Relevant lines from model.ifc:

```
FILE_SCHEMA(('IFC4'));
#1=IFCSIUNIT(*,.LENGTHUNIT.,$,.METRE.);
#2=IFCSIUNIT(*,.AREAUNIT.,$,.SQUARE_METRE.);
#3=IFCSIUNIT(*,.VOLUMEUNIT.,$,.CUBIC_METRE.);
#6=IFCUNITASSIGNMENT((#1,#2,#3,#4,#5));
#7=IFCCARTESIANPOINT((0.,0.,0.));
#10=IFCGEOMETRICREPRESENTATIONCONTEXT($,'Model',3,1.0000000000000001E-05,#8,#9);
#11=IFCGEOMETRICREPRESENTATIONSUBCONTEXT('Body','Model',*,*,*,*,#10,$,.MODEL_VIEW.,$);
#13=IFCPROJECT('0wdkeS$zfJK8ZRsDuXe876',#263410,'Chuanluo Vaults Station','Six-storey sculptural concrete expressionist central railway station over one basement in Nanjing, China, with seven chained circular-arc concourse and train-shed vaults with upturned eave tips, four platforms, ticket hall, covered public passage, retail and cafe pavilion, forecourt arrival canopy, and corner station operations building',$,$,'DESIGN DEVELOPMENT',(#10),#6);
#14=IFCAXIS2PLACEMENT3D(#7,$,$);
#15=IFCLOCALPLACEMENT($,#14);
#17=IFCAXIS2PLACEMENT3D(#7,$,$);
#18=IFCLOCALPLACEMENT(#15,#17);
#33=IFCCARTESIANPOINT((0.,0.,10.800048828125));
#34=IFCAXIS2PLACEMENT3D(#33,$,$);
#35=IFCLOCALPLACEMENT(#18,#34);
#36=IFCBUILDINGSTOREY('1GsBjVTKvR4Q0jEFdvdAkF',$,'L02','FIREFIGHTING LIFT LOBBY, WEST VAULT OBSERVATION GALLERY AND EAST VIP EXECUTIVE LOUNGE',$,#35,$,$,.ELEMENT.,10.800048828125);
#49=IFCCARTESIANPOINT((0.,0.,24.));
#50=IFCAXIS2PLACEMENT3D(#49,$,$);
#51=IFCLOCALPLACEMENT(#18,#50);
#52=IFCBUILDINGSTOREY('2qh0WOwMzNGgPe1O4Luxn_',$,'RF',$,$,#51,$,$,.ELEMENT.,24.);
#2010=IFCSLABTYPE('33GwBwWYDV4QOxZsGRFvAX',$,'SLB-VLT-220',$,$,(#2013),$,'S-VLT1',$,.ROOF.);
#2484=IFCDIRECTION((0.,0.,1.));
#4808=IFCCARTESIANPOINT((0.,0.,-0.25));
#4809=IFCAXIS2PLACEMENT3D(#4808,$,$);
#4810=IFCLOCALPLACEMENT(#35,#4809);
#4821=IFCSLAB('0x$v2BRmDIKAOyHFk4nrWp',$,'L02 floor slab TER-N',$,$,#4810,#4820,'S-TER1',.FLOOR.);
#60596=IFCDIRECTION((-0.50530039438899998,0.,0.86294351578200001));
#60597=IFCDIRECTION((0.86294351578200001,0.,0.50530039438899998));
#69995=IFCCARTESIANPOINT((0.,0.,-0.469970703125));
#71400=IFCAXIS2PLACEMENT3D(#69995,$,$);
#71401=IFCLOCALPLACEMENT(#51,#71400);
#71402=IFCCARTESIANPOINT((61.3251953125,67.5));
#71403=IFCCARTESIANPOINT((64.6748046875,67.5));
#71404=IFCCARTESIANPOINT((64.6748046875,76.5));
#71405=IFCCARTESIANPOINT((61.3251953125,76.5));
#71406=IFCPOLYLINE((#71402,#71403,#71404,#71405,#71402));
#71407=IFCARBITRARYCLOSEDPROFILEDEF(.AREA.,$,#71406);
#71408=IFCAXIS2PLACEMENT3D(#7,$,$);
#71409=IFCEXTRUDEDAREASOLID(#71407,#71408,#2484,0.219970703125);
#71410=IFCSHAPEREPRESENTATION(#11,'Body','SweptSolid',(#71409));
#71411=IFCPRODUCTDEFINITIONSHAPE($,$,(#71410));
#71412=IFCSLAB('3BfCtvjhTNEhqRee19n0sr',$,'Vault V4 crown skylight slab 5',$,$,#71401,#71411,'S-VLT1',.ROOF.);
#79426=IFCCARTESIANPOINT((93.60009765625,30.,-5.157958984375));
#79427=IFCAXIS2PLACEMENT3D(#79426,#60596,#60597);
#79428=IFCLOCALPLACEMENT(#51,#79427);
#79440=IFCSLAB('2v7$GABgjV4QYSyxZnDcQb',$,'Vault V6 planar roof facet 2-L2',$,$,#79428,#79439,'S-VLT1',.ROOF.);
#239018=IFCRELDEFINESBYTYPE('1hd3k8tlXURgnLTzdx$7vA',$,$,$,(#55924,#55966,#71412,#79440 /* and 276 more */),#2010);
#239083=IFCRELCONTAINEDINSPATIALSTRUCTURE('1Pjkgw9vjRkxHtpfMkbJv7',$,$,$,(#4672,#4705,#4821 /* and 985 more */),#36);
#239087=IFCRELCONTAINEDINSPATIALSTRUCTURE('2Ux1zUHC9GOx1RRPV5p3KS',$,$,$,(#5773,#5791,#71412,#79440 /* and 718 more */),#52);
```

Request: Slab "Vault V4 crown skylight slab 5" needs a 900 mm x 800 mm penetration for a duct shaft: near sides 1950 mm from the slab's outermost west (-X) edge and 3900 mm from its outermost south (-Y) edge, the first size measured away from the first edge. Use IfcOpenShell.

```python
import numpy as np
import ifcopenshell
import ifcopenshell.api.feature
import ifcopenshell.api.geometry
import ifcopenshell.api.root
import ifcopenshell.geom
import ifcopenshell.util.placement
import ifcopenshell.util.representation
import ifcopenshell.util.shape
import ifcopenshell.util.unit

model = ifcopenshell.open("model.ifc")
unit_scale = ifcopenshell.util.unit.calculate_unit_scale(model)
settings = ifcopenshell.geom.settings()


def volume(element):
    """Net volume in cubic metres, openings subtracted."""
    shape = ifcopenshell.geom.create_shape(settings, element)
    return ifcopenshell.util.shape.get_volume(shape.geometry)


slab = model.by_guid("3BfCtvjhTNEhqRee19n0sr")
before = volume(slab)

# Extent in the slab's own axes, in metres. The edges named are its -X and -Y sides.
slab_shape = ifcopenshell.geom.create_shape(settings, slab)
vertices = ifcopenshell.util.shape.get_vertices(slab_shape.geometry)
x_min, y_min, bottom = vertices.min(axis=0)
top = vertices[:, 2].max()

opening = ifcopenshell.api.root.create_entity(model, ifc_class="IfcOpeningElement", name="Duct shaft opening", predefined_type="OPENING")
context = ifcopenshell.util.representation.get_context(model, "Model", "Body", "MODEL_VIEW")
width, depth = 0.9, 0.8
outline = [(0.0, 0.0), (width, 0.0), (width, depth), (0.0, depth), (0.0, 0.0)]
# Overshoot both faces by 50 mm so the cut is clean.
shape = ifcopenshell.api.geometry.add_slab_representation(
    model, context=context, depth=top - bottom + 0.1, polyline=outline
)
ifcopenshell.api.geometry.assign_representation(model, product=opening, representation=shape)

matrix = ifcopenshell.util.placement.get_local_placement(slab.ObjectPlacement)
matrix[:, 3] = matrix @ np.append(np.array([x_min + 1.95, y_min + 3.9, bottom - 0.05]) / unit_scale, 1.0)
ifcopenshell.api.geometry.edit_object_placement(model, product=opening, matrix=matrix, is_si=False)
ifcopenshell.api.feature.add_feature(model, feature=opening, element=slab)

after = volume(slab)

print(f"slab volume {before:.3f} -> {after:.3f} m3")

model.write("model_updated.ifc")
```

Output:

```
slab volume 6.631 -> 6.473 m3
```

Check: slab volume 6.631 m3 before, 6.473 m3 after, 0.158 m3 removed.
